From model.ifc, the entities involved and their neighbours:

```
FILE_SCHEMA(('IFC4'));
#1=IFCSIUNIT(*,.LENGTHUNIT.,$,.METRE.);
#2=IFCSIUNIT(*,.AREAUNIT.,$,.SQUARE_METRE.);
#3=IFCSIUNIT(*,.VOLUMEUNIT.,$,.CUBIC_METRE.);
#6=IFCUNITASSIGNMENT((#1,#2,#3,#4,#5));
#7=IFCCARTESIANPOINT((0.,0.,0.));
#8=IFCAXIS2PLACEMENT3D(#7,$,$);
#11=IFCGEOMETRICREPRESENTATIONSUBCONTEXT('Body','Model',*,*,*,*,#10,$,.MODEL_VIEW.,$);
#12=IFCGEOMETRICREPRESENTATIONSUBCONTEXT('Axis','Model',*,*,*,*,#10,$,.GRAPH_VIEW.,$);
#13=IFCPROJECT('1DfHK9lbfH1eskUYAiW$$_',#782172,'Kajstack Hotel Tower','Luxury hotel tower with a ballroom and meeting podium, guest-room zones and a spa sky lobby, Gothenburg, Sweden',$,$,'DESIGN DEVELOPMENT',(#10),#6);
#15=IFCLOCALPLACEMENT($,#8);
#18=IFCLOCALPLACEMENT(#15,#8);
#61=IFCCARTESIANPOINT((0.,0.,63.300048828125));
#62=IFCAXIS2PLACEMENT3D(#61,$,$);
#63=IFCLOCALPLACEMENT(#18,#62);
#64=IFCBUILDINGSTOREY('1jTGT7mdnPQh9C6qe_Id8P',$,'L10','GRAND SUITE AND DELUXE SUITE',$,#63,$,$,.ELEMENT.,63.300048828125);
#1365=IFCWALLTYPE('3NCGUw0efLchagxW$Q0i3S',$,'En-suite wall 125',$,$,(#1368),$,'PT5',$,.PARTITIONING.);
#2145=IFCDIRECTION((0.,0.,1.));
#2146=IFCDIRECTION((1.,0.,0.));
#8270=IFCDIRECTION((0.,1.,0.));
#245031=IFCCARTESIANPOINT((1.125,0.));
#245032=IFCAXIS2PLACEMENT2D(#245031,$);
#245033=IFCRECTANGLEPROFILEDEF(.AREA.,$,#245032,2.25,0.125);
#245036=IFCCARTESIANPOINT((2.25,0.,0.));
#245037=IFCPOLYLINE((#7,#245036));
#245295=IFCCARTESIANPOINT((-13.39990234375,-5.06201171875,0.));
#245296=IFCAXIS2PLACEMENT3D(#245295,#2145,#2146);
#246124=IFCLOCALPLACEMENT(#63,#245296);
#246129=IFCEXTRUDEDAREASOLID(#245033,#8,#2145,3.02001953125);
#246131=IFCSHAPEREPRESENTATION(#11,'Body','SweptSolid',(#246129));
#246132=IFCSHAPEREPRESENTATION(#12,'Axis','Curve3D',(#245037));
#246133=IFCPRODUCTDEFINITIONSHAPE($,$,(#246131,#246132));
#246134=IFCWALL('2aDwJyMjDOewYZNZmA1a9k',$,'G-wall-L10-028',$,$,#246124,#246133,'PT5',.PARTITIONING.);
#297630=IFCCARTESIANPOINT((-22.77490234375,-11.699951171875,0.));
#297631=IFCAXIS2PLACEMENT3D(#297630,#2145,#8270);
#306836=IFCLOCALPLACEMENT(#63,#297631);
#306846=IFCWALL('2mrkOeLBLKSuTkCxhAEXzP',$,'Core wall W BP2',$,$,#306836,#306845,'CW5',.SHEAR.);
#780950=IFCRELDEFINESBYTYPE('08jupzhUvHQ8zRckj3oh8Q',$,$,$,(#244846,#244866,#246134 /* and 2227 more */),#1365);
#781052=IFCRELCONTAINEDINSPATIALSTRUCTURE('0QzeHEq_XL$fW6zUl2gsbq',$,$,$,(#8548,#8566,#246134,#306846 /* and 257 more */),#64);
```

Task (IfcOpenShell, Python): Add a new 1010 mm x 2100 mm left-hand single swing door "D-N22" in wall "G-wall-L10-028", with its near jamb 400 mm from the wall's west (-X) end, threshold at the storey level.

```python
import numpy as np
import ifcopenshell
import ifcopenshell.api.feature
import ifcopenshell.api.geometry
import ifcopenshell.api.root
import ifcopenshell.api.spatial
import ifcopenshell.geom
import ifcopenshell.util.element
import ifcopenshell.util.placement
import ifcopenshell.util.representation
import ifcopenshell.util.shape
import ifcopenshell.util.unit

model = ifcopenshell.open("model.ifc")
unit_scale = ifcopenshell.util.unit.calculate_unit_scale(model)
settings = ifcopenshell.geom.settings()


def volume(element):
    """Net volume in cubic metres, openings subtracted."""
    shape = ifcopenshell.geom.create_shape(settings, element)
    return ifcopenshell.util.shape.get_volume(shape.geometry)


wall = model.by_guid("2aDwJyMjDOewYZNZmA1a9k")
storey = ifcopenshell.util.element.get_container(wall, ifc_class="IfcBuildingStorey")
context = ifcopenshell.util.representation.get_context(model, "Model", "Body", "MODEL_VIEW")
before = volume(wall)

width, height, from_end, sill = 1.01, 2.1, 0.4, 0.0  # metres

# The wall runs along its own X axis, and the end named is its -X end.
wall_shape = ifcopenshell.geom.create_shape(settings, wall)
x, y, z = ifcopenshell.util.shape.get_vertices(wall_shape.geometry).T
start = x.min() + from_end
face, thickness = float(y.min()), float(y.max() - y.min())
wall_matrix = ifcopenshell.util.placement.get_local_placement(wall.ObjectPlacement)
level = ifcopenshell.util.placement.get_local_placement(storey.ObjectPlacement)[2, 3]


def in_wall(x, y):
    """Placement at x, y metres in the wall's axes, at sill height."""
    matrix = wall_matrix.copy()
    matrix[:, 3] = wall_matrix @ np.array([x / unit_scale, y / unit_scale, 0.0, 1.0])
    matrix[2, 3] = level + sill / unit_scale
    return matrix


# Opening: a box that overshoots both wall faces by 50 mm.
opening = ifcopenshell.api.root.create_entity(model, ifc_class="IfcOpeningElement", predefined_type="OPENING")
box = ifcopenshell.api.geometry.add_wall_representation(
    model, context=context, length=width, height=height, thickness=thickness + 0.1
)
ifcopenshell.api.geometry.assign_representation(model, product=opening, representation=box)
ifcopenshell.api.geometry.edit_object_placement(model, product=opening, matrix=in_wall(start, face - 0.05), is_si=False)
ifcopenshell.api.feature.add_feature(model, feature=opening, element=wall)

door = ifcopenshell.api.root.create_entity(model, ifc_class="IfcDoor", name="D-N22", predefined_type="DOOR")
door.OverallWidth, door.OverallHeight = width / unit_scale, height / unit_scale
door.OperationType = "SINGLE_SWING_LEFT"
body = ifcopenshell.api.geometry.add_door_representation(
    model,
    context=context,
    overall_width=door.OverallWidth,
    overall_height=door.OverallHeight,
    operation_type="SINGLE_SWING_LEFT",
    lining_properties={"LiningDepth": thickness / unit_scale, "ThresholdDepth": thickness / unit_scale},
)
ifcopenshell.api.geometry.assign_representation(model, product=door, representation=body)
ifcopenshell.api.spatial.assign_container(model, products=[door], relating_structure=storey)
ifcopenshell.api.feature.add_filling(model, opening=opening, element=door)

# The lining spans the wall, so the door starts at the wall face.
ifcopenshell.api.geometry.edit_object_placement(model, product=door, matrix=in_wall(start, face), is_si=False)

after = volume(wall)

print(f"wall volume {before:.3f} -> {after:.3f} m3")

model.write("model-out.ifc")
```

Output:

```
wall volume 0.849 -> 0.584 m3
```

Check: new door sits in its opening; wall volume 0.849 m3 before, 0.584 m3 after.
